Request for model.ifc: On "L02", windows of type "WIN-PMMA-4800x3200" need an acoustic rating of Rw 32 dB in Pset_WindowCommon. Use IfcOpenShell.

First a look at what the model holds.

```python
import ifcopenshell
import ifcopenshell.util.element

model = ifcopenshell.open("model.ifc")
print(model.schema)
storey = next(s for s in model.by_type("IfcBuildingStorey") if s.Name == "L02")
windows = [e for e in ifcopenshell.util.element.get_decomposition(storey) if e.is_a("IfcWindow")]
seen = {}
for e in windows:
    element_type = ifcopenshell.util.element.get_type(e)
    key = (element_type.Name if element_type != e and element_type else None, ifcopenshell.util.element.get_pset(e, "Pset_WindowCommon", "AcousticRating"))
    seen[key] = seen.get(key, 0) + 1
for (name, value), count in sorted(seen.items(), key=str):
    print(count, "x", name, "|", value)
```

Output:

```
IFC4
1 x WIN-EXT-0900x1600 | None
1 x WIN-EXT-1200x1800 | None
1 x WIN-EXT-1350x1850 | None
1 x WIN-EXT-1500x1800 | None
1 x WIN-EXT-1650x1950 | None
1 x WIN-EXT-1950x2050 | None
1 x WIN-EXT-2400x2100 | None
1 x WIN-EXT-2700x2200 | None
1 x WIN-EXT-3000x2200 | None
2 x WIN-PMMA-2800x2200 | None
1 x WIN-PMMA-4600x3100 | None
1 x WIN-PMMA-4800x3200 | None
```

```python
import ifcopenshell
import ifcopenshell.api.pset
import ifcopenshell.util.element

model = ifcopenshell.open("model.ifc")

storey = next(s for s in model.by_type("IfcBuildingStorey") if s.Name == "L02")
windows = [e for e in ifcopenshell.util.element.get_decomposition(storey) if e.is_a("IfcWindow")]

count = 0
for e in windows:
    element_type = ifcopenshell.util.element.get_type(e)
    if element_type in (None, e) or element_type.Name != "WIN-PMMA-4800x3200":
        continue
    # add_pset returns the element's existing set when there is one.
    pset = ifcopenshell.api.pset.add_pset(model, product=e, name="Pset_WindowCommon")
    ifcopenshell.api.pset.edit_pset(model, pset=pset, properties={"AcousticRating": "Rw 32 dB"})
    count += 1

print(count, "windows updated")

model.write("model_edited.ifc")
```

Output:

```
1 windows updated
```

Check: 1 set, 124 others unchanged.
